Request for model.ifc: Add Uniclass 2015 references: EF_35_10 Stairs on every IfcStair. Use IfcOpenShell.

First a look at what the model holds.

```python
import ifcopenshell

model = ifcopenshell.open("model.ifc")
print(model.schema)
print("classifications:", [c.Name for c in model.by_type("IfcClassification")])
for ifc_class in ("IfcDoor", "IfcRoof", "IfcStair", "IfcWall", "IfcWindow"):
    print(ifc_class, len(model.by_type(ifc_class)))
```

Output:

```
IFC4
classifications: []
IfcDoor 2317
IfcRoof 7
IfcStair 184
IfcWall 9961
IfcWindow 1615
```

```python
import ifcopenshell
import ifcopenshell.api.classification

model = ifcopenshell.open("model.ifc")

system = ifcopenshell.api.classification.add_classification(model, classification="Uniclass 2015")

codes = {
    "IfcStair": ("EF_35_10", "Stairs"),
}
for ifc_class, (code, name) in codes.items():
    products = model.by_type(ifc_class)
    ifcopenshell.api.classification.add_reference(
        model, products=products, classification=system, identification=code, name=name
    )
    print(code, len(products))

model.write("model_rev.ifc")
```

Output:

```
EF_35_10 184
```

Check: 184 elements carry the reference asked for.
